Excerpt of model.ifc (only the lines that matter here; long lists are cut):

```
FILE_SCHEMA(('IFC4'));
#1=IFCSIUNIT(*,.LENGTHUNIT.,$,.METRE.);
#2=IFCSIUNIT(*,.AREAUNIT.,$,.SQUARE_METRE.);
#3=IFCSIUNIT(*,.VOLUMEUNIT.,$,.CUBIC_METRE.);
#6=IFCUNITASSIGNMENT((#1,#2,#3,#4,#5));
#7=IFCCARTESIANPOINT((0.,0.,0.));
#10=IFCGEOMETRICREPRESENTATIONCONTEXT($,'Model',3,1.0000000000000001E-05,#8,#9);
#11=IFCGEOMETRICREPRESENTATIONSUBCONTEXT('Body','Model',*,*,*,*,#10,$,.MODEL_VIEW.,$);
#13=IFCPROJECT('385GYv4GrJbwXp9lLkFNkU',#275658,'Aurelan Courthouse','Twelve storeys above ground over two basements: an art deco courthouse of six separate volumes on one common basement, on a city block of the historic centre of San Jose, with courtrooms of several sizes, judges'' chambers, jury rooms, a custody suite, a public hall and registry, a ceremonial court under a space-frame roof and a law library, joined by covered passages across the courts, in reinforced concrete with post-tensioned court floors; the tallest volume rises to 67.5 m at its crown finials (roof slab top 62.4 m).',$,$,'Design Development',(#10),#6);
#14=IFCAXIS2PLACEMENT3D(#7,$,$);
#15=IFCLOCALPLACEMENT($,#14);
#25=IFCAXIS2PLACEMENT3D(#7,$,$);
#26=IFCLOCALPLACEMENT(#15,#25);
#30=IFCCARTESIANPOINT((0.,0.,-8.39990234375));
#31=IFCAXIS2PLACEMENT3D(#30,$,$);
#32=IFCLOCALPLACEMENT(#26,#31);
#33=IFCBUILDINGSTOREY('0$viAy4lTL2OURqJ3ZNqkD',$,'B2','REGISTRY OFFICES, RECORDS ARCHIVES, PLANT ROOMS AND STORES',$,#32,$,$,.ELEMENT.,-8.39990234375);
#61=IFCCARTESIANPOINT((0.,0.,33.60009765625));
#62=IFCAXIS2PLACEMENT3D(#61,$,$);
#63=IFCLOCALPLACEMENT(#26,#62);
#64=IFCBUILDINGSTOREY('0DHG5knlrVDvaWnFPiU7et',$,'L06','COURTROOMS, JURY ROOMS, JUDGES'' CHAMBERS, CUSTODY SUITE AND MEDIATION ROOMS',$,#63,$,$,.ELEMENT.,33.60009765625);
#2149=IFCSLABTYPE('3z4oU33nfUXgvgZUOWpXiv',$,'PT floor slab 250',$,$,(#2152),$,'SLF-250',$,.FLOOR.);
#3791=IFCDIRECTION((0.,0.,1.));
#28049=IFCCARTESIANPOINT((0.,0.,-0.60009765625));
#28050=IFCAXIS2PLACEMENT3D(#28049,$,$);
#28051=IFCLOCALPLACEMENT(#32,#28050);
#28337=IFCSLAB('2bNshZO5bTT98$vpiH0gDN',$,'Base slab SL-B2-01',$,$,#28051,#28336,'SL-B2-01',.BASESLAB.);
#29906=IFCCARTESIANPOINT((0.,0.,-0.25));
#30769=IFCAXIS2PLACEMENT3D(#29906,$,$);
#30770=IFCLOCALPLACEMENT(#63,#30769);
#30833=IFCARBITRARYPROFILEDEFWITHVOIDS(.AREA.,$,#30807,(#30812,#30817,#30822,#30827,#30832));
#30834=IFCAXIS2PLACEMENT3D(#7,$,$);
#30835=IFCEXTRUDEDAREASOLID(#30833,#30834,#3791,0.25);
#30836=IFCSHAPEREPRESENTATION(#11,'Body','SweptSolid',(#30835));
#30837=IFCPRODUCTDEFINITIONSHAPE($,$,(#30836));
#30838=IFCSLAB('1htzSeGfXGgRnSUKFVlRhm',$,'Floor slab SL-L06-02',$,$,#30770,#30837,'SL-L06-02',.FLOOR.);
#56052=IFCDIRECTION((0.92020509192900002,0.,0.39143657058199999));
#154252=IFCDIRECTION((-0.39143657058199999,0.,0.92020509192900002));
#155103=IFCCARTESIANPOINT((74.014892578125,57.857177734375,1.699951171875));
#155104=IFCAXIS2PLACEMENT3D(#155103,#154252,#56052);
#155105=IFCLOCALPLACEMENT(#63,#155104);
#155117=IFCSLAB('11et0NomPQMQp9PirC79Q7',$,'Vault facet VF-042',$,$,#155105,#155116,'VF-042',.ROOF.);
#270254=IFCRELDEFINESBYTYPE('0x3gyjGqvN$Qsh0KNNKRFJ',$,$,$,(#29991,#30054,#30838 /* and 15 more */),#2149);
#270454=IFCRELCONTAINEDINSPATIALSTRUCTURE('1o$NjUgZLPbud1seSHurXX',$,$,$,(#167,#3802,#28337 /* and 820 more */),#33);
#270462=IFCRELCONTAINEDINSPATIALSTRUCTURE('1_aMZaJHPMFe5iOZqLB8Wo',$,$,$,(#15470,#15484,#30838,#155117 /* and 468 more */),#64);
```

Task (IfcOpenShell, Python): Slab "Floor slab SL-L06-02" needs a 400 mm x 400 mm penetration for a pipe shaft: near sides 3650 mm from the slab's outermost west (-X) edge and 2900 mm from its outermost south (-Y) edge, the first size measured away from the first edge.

```python
import numpy as np
import ifcopenshell
import ifcopenshell.api.feature
import ifcopenshell.api.geometry
import ifcopenshell.api.root
import ifcopenshell.geom
import ifcopenshell.util.placement
import ifcopenshell.util.representation
import ifcopenshell.util.shape
import ifcopenshell.util.unit

model = ifcopenshell.open("model.ifc")
unit_scale = ifcopenshell.util.unit.calculate_unit_scale(model)
settings = ifcopenshell.geom.settings()


def volume(element):
    """Net volume in cubic metres, openings subtracted."""
    shape = ifcopenshell.geom.create_shape(settings, element)
    return ifcopenshell.util.shape.get_volume(shape.geometry)


slab = model.by_id(30838)
before = volume(slab)

# Extent in the slab's own axes, in metres. The edges named are its -X and -Y sides.
slab_shape = ifcopenshell.geom.create_shape(settings, slab)
vertices = ifcopenshell.util.shape.get_vertices(slab_shape.geometry)
x_min, y_min, bottom = vertices.min(axis=0)
top = vertices[:, 2].max()

opening = ifcopenshell.api.root.create_entity(model, ifc_class="IfcOpeningElement", name="Pipe shaft opening", predefined_type="OPENING")
context = ifcopenshell.util.representation.get_context(model, "Model", "Body", "MODEL_VIEW")
width, depth = 0.4, 0.4
outline = [(0.0, 0.0), (width, 0.0), (width, depth), (0.0, depth), (0.0, 0.0)]
# Overshoot both faces by 50 mm so the cut is clean.
shape = ifcopenshell.api.geometry.add_slab_representation(
    model, context=context, depth=top - bottom + 0.1, polyline=outline
)
ifcopenshell.api.geometry.assign_representation(model, product=opening, representation=shape)

matrix = ifcopenshell.util.placement.get_local_placement(slab.ObjectPlacement)
matrix[:, 3] = matrix @ np.append(np.array([x_min + 3.65, y_min + 2.9, bottom - 0.05]) / unit_scale, 1.0)
ifcopenshell.api.geometry.edit_object_placement(model, product=opening, matrix=matrix, is_si=False)
ifcopenshell.api.feature.add_feature(model, feature=opening, element=slab)

after = volume(slab)

print(f"slab volume {before:.3f} -> {after:.3f} m3")

model.write("model-out.ifc")
```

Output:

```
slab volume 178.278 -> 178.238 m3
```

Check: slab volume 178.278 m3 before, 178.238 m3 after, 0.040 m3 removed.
